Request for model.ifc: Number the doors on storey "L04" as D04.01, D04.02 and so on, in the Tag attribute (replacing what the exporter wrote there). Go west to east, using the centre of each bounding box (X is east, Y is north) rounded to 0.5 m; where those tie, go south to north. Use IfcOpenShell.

First a look at what the model holds.

```python
import ifcopenshell
import ifcopenshell.util.element
import ifcopenshell.util.placement

model = ifcopenshell.open("model.ifc")
print(model.schema)
storey = next(s for s in model.by_type("IfcBuildingStorey") if s.Name == "L04")
doors = [e for e in ifcopenshell.util.element.get_decomposition(storey) if e.is_a("IfcDoor")]
for e in sorted(doors, key=lambda e: e.id()):
    origin = ifcopenshell.util.placement.get_local_placement(e.ObjectPlacement)[:3, 3]
    print(e.id(), e.Tag, e.Name, origin.round(2) + 0.0, sep=" | ")
```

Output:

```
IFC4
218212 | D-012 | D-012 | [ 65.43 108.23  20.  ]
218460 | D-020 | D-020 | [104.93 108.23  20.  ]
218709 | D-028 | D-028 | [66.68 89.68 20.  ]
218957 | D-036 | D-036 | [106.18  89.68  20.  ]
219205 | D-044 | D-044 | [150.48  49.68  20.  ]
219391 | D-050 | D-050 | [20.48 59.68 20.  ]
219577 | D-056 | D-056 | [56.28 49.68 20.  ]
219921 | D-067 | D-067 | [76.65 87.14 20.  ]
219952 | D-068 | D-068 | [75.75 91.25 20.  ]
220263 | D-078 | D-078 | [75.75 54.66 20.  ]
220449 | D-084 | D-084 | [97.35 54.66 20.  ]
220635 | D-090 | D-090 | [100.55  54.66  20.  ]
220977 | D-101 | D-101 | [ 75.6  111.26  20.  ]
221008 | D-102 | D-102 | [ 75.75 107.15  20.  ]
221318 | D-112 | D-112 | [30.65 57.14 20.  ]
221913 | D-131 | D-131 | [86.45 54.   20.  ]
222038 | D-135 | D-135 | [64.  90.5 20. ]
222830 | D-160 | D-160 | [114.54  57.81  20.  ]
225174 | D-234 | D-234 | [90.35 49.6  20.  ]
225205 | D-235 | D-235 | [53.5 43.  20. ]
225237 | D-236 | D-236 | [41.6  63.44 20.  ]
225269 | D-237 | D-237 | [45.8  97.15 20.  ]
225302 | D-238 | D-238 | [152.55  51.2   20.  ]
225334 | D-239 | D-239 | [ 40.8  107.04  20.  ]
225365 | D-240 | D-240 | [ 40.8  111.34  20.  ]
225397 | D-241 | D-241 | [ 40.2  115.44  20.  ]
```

```python
import ifcopenshell
import ifcopenshell.geom
import ifcopenshell.util.element
import ifcopenshell.util.shape

model = ifcopenshell.open("model.ifc")
settings = ifcopenshell.geom.settings()
settings.set("use-world-coords", True)


def centre(element):
    shape = ifcopenshell.geom.create_shape(settings, element)
    return ifcopenshell.util.shape.get_bbox_centroid(shape.geometry)


storey = next(s for s in model.by_type("IfcBuildingStorey") if s.Name == "L04")
doors = [e for e in ifcopenshell.util.element.get_decomposition(storey) if e.is_a("IfcDoor")]

# Insertion points can sit at a corner or the storey origin, so sort by the geometry (in metres).
centres = {e: centre(e) for e in doors}
doors.sort(key=lambda e: (round(centres[e][0] / 0.5), centres[e][1]))

for i, e in enumerate(doors, start=1):
    number = f"D04.{i:02d}"
    e.Tag = number
    print(e.id(), number)

model.write("model_updated.ifc")
```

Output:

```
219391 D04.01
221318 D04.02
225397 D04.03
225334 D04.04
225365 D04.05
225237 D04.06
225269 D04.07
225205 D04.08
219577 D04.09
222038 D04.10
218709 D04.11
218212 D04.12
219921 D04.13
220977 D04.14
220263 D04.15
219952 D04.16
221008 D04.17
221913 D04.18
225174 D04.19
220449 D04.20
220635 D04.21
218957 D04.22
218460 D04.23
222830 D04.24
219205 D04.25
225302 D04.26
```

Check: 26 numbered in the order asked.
